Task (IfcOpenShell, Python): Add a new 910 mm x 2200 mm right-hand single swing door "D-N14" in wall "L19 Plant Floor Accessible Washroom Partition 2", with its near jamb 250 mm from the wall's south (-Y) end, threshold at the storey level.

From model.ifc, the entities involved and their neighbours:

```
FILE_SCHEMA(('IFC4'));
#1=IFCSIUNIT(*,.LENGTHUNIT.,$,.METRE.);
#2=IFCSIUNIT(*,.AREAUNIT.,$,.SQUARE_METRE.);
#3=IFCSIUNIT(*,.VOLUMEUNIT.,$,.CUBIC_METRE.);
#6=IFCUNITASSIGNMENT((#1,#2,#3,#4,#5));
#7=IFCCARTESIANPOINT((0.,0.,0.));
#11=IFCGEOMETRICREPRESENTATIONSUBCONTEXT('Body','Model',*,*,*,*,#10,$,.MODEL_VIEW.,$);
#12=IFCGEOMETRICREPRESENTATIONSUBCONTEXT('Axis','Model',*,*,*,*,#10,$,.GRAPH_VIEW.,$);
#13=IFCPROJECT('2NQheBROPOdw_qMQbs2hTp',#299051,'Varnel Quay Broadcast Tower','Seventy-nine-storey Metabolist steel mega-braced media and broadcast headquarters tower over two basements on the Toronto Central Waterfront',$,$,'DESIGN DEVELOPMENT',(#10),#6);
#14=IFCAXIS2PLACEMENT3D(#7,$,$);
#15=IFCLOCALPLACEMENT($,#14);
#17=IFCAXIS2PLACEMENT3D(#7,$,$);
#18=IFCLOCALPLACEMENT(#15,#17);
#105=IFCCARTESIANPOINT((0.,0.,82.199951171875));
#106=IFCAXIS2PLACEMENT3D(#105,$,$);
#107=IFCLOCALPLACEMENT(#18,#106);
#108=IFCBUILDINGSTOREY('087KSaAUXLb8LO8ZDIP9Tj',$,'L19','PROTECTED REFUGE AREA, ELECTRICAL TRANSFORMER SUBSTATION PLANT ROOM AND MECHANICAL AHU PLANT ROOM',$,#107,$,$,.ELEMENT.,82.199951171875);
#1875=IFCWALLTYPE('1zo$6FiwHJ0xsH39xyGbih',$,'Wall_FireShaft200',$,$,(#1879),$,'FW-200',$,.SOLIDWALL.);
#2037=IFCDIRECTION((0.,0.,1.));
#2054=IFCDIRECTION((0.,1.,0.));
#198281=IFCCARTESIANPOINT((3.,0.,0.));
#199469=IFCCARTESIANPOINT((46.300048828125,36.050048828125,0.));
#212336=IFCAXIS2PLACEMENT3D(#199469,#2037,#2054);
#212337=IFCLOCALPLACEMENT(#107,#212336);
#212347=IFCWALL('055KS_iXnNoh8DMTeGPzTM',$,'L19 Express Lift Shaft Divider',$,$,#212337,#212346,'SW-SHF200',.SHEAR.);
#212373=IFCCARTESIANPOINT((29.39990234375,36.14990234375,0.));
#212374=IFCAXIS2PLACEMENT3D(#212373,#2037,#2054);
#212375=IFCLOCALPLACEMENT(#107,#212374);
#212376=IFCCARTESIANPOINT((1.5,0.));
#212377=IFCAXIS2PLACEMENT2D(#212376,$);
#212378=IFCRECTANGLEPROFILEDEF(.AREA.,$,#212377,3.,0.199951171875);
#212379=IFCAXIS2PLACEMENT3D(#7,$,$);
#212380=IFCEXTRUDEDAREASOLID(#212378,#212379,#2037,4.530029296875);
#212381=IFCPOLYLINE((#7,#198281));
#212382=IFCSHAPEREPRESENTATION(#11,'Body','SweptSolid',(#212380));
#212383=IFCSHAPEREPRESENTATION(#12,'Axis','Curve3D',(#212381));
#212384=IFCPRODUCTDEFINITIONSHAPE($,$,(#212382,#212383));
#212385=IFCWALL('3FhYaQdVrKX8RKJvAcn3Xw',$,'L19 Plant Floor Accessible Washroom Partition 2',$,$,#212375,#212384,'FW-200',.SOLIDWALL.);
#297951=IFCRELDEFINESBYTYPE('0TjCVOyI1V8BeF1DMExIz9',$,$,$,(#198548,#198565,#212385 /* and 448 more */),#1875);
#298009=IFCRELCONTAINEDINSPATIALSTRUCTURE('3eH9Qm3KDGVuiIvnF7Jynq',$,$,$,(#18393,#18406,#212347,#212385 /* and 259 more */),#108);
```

```python
import numpy as np
import ifcopenshell
import ifcopenshell.api.feature
import ifcopenshell.api.geometry
import ifcopenshell.api.root
import ifcopenshell.api.spatial
import ifcopenshell.geom
import ifcopenshell.util.element
import ifcopenshell.util.placement
import ifcopenshell.util.representation
import ifcopenshell.util.shape
import ifcopenshell.util.unit

model = ifcopenshell.open("model.ifc")
unit_scale = ifcopenshell.util.unit.calculate_unit_scale(model)
settings = ifcopenshell.geom.settings()


def volume(element):
    """Net volume in cubic metres, openings subtracted."""
    shape = ifcopenshell.geom.create_shape(settings, element)
    return ifcopenshell.util.shape.get_volume(shape.geometry)


wall = model.by_id(212385)
storey = ifcopenshell.util.element.get_container(wall, ifc_class="IfcBuildingStorey")
context = ifcopenshell.util.representation.get_context(model, "Model", "Body", "MODEL_VIEW")
before = volume(wall)

width, height, from_end, sill = 0.91, 2.2, 0.25, 0.0  # metres

# The wall runs along its own X axis, and the end named is its -X end.
wall_shape = ifcopenshell.geom.create_shape(settings, wall)
x, y, z = ifcopenshell.util.shape.get_vertices(wall_shape.geometry).T
start = x.min() + from_end
face, thickness = float(y.min()), float(y.max() - y.min())
wall_matrix = ifcopenshell.util.placement.get_local_placement(wall.ObjectPlacement)
level = ifcopenshell.util.placement.get_local_placement(storey.ObjectPlacement)[2, 3]


def in_wall(x, y):
    """Placement at x, y metres in the wall's axes, at sill height."""
    matrix = wall_matrix.copy()
    matrix[:, 3] = wall_matrix @ np.array([x / unit_scale, y / unit_scale, 0.0, 1.0])
    matrix[2, 3] = level + sill / unit_scale
    return matrix


# Opening: a box that overshoots both wall faces by 50 mm.
opening = ifcopenshell.api.root.create_entity(model, ifc_class="IfcOpeningElement", predefined_type="OPENING")
box = ifcopenshell.api.geometry.add_wall_representation(
    model, context=context, length=width, height=height, thickness=thickness + 0.1
)
ifcopenshell.api.geometry.assign_representation(model, product=opening, representation=box)
ifcopenshell.api.geometry.edit_object_placement(model, product=opening, matrix=in_wall(start, face - 0.05), is_si=False)
ifcopenshell.api.feature.add_feature(model, feature=opening, element=wall)

door = ifcopenshell.api.root.create_entity(model, ifc_class="IfcDoor", name="D-N14", predefined_type="DOOR")
door.OverallWidth, door.OverallHeight = width / unit_scale, height / unit_scale
door.OperationType = "SINGLE_SWING_RIGHT"
body = ifcopenshell.api.geometry.add_door_representation(
    model,
    context=context,
    overall_width=door.OverallWidth,
    overall_height=door.OverallHeight,
    operation_type="SINGLE_SWING_RIGHT",
    lining_properties={"LiningDepth": thickness / unit_scale, "ThresholdDepth": thickness / unit_scale},
)
ifcopenshell.api.geometry.assign_representation(model, product=door, representation=body)
ifcopenshell.api.spatial.assign_container(model, products=[door], relating_structure=storey)
ifcopenshell.api.feature.add_filling(model, opening=opening, element=door)

# The lining spans the wall, so the door starts at the wall face.
ifcopenshell.api.geometry.edit_object_placement(model, product=door, matrix=in_wall(start, face), is_si=False)

after = volume(wall)

print(f"wall volume {before:.3f} -> {after:.3f} m3")

model.write("model_edited.ifc")
```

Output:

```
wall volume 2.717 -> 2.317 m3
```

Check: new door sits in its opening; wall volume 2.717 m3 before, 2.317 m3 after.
